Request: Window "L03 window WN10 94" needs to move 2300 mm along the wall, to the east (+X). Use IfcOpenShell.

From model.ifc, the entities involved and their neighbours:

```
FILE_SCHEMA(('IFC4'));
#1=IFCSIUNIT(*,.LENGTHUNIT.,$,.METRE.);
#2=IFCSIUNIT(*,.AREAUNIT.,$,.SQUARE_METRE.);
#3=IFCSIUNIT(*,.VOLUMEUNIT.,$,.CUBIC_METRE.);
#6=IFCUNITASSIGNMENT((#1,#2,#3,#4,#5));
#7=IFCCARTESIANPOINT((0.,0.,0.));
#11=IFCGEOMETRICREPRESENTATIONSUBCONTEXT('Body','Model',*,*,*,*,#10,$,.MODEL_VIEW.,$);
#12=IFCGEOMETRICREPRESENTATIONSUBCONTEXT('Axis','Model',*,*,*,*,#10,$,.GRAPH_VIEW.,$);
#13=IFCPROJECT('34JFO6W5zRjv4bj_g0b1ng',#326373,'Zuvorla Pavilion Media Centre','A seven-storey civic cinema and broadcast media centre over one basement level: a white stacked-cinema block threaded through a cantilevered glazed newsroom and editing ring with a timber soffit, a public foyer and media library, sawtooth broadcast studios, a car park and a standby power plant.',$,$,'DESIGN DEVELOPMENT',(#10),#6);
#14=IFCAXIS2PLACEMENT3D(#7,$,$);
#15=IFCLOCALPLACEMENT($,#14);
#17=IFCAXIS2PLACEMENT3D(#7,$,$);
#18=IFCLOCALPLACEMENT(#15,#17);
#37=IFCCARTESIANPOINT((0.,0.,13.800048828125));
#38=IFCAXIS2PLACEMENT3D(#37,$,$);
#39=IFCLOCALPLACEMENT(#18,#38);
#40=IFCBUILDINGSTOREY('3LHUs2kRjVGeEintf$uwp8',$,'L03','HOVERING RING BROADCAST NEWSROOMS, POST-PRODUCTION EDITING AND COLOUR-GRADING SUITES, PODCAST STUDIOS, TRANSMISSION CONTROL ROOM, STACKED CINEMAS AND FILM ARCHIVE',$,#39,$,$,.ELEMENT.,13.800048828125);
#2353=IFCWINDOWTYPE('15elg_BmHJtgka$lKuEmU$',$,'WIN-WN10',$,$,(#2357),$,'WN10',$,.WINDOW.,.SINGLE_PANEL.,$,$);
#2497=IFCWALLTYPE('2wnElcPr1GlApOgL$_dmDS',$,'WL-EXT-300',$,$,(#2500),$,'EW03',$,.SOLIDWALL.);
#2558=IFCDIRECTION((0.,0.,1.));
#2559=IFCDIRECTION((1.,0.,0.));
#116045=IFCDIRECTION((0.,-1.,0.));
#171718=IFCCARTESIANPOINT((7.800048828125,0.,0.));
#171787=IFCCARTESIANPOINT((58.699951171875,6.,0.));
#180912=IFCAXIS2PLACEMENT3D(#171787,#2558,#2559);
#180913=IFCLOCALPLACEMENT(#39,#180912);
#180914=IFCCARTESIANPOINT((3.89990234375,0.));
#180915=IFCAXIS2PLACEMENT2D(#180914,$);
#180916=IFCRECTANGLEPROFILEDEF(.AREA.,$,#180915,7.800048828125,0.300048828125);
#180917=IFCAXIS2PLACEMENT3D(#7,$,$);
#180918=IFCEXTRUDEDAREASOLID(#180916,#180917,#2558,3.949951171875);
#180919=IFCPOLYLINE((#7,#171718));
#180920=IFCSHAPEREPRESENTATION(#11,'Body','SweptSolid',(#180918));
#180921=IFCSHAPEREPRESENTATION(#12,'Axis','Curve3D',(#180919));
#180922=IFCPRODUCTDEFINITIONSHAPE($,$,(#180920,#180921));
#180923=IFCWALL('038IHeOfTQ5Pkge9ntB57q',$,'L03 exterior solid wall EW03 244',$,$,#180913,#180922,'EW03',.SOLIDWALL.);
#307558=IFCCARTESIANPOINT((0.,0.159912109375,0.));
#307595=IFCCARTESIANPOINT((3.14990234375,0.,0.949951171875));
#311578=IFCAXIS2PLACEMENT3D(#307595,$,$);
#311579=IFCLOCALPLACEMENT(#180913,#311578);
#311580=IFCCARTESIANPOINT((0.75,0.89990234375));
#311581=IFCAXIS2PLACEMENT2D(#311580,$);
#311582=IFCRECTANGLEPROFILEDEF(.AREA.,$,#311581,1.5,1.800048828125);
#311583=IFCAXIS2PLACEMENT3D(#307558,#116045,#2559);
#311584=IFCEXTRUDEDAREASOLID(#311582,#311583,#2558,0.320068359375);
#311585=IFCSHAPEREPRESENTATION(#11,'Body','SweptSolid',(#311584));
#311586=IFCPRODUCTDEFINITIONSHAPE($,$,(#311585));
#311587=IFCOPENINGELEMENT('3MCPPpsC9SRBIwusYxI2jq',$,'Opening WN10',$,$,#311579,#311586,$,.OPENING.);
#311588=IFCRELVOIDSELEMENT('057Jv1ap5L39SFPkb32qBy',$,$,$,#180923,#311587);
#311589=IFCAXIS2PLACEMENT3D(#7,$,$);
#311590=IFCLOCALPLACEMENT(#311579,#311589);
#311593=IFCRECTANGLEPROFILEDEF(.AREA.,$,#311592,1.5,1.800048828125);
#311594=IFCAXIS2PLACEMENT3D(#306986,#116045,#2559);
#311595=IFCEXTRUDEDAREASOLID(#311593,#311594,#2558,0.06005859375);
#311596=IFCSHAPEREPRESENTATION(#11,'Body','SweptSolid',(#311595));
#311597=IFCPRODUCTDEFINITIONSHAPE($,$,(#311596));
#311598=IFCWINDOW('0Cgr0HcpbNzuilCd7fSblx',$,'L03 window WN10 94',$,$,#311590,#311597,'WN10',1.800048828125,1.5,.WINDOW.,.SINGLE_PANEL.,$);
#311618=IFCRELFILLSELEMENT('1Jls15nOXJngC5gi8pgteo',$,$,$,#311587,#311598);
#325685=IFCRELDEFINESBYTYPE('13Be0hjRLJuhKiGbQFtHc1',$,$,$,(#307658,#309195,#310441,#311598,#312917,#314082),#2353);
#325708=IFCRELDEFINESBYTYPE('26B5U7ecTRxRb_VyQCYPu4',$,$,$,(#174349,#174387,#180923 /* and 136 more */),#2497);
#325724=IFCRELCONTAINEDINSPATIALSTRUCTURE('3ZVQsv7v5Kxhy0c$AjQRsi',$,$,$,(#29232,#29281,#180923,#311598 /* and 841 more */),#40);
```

```python
import ifcopenshell
import ifcopenshell.api.geometry
import ifcopenshell.util.placement
import ifcopenshell.util.unit

model = ifcopenshell.open("model.ifc")
unit_scale = ifcopenshell.util.unit.calculate_unit_scale(model)

window = model.by_id(311598)
opening = window.FillsVoids[0].RelatingOpeningElement
wall = opening.VoidsElements[0].RelatingBuildingElement

wall_matrix = ifcopenshell.util.placement.get_local_placement(wall.ObjectPlacement)
shift = wall_matrix[:3, 0] * 2.3 / unit_scale
before = ifcopenshell.util.placement.get_local_placement(window.ObjectPlacement)[:3, 3].copy()

# The window is placed relative to its opening, so it follows when the opening moves.
matrix = ifcopenshell.util.placement.get_local_placement(opening.ObjectPlacement)
matrix[:3, 3] += shift
ifcopenshell.api.geometry.edit_object_placement(
    model, product=opening, matrix=matrix, is_si=False, should_transform_children=True
)

after = ifcopenshell.util.placement.get_local_placement(window.ObjectPlacement)[:3, 3]
print("window moved by", (after - before).round(3) + 0.0)

model.write("model_updated.ifc")
```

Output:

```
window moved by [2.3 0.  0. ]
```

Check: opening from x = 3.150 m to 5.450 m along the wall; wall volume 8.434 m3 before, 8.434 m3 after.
